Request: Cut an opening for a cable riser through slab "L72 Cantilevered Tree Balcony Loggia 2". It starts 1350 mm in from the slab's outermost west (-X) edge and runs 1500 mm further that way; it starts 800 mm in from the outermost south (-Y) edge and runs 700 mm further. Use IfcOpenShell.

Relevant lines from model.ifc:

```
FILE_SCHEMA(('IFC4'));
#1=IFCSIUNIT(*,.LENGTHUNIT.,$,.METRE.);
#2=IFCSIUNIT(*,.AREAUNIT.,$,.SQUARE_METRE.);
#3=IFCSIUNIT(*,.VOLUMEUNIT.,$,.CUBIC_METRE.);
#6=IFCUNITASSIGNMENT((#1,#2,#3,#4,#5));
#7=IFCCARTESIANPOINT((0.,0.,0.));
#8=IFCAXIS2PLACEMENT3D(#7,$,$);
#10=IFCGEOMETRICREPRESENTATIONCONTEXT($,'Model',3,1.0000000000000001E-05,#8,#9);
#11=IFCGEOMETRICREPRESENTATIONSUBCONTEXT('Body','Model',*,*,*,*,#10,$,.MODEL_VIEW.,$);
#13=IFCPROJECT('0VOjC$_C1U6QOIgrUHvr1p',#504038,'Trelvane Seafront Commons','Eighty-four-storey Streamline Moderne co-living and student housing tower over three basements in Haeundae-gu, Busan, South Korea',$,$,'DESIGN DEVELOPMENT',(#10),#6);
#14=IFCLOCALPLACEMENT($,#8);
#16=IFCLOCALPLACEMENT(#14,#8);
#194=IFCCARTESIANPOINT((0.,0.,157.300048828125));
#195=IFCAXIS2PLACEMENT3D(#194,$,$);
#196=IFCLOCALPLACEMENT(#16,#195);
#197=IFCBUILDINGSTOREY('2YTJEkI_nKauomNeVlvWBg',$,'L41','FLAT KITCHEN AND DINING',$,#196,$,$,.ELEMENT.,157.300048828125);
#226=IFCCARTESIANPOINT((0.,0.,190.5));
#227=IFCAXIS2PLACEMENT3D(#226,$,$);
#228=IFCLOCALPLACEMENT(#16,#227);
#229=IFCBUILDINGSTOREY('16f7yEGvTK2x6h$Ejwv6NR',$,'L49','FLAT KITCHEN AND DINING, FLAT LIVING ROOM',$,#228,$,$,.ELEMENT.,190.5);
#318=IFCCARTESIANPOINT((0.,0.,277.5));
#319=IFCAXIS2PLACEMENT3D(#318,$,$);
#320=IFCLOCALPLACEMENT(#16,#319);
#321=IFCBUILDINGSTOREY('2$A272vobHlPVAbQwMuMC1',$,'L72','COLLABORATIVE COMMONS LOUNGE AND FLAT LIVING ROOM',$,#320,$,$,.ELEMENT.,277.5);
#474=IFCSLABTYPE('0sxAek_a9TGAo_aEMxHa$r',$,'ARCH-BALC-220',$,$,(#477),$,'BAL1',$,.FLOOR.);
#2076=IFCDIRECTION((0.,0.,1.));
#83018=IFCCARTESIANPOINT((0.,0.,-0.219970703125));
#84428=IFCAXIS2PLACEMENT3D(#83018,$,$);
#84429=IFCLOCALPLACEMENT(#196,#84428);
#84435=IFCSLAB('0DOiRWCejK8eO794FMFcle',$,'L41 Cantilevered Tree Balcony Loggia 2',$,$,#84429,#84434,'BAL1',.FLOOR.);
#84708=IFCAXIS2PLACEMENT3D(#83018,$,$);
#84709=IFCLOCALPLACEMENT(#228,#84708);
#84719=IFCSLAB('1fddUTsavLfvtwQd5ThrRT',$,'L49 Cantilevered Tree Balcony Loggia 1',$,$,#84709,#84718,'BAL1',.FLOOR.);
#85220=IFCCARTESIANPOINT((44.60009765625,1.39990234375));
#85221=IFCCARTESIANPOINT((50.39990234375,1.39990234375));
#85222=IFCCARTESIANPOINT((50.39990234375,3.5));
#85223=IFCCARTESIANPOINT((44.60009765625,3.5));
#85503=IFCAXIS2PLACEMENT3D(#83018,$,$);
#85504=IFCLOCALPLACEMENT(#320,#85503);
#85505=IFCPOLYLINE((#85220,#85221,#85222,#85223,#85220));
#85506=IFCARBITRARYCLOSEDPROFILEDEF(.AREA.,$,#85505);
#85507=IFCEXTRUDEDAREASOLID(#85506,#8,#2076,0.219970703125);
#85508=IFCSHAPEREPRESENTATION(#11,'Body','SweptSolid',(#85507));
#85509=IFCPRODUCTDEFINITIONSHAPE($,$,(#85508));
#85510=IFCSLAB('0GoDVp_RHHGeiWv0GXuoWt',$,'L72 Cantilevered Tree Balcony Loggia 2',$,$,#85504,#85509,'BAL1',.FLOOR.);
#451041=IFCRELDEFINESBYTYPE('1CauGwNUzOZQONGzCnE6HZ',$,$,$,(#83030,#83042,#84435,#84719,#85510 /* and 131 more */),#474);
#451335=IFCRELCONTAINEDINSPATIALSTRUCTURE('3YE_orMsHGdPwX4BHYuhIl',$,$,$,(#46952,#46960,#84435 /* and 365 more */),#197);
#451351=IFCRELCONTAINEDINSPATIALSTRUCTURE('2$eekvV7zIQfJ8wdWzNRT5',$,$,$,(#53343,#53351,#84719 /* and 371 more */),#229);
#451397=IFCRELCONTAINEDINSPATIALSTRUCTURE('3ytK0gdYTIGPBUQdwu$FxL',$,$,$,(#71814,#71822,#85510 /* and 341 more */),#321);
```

```python
import numpy as np
import ifcopenshell
import ifcopenshell.api.feature
import ifcopenshell.api.geometry
import ifcopenshell.api.root
import ifcopenshell.geom
import ifcopenshell.util.placement
import ifcopenshell.util.representation
import ifcopenshell.util.shape
import ifcopenshell.util.unit

model = ifcopenshell.open("model.ifc")
unit_scale = ifcopenshell.util.unit.calculate_unit_scale(model)
settings = ifcopenshell.geom.settings()


def volume(element):
    """Net volume in cubic metres, openings subtracted."""
    shape = ifcopenshell.geom.create_shape(settings, element)
    return ifcopenshell.util.shape.get_volume(shape.geometry)


slab = model.by_guid("0GoDVp_RHHGeiWv0GXuoWt")
before = volume(slab)

# Extent in the slab's own axes, in metres. The edges named are its -X and -Y sides.
slab_shape = ifcopenshell.geom.create_shape(settings, slab)
vertices = ifcopenshell.util.shape.get_vertices(slab_shape.geometry)
x_min, y_min, bottom = vertices.min(axis=0)
top = vertices[:, 2].max()

opening = ifcopenshell.api.root.create_entity(model, ifc_class="IfcOpeningElement", name="Cable riser opening", predefined_type="OPENING")
context = ifcopenshell.util.representation.get_context(model, "Model", "Body", "MODEL_VIEW")
width, depth = 1.5, 0.7
outline = [(0.0, 0.0), (width, 0.0), (width, depth), (0.0, depth), (0.0, 0.0)]
# Overshoot both faces by 50 mm so the cut is clean.
shape = ifcopenshell.api.geometry.add_slab_representation(
    model, context=context, depth=top - bottom + 0.1, polyline=outline
)
ifcopenshell.api.geometry.assign_representation(model, product=opening, representation=shape)

matrix = ifcopenshell.util.placement.get_local_placement(slab.ObjectPlacement)
matrix[:, 3] = matrix @ np.append(np.array([x_min + 1.35, y_min + 0.8, bottom - 0.05]) / unit_scale, 1.0)
ifcopenshell.api.geometry.edit_object_placement(model, product=opening, matrix=matrix, is_si=False)
ifcopenshell.api.feature.add_feature(model, feature=opening, element=slab)

after = volume(slab)

print(f"slab volume {before:.3f} -> {after:.3f} m3")

model.write("model_rev.ifc")
```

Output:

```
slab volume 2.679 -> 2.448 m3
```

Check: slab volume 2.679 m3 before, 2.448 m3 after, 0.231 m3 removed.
